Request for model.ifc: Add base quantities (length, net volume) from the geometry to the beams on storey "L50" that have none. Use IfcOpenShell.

First a look at what the model holds.

```python
import ifcopenshell
import ifcopenshell.util.element
import ifcopenshell.util.unit

model = ifcopenshell.open("model.ifc")
print(model.schema)
for unit_type in ("LENGTHUNIT", "AREAUNIT", "VOLUMEUNIT"):
    print(unit_type, ifcopenshell.util.unit.calculate_unit_scale(model, unit_type))
storey = next(s for s in model.by_type("IfcBuildingStorey") if s.Name == "L50")
beams = [e for e in ifcopenshell.util.element.get_decomposition(storey) if e.is_a("IfcBeam")]
for e in sorted(beams, key=lambda e: e.id()):
    print(e.id(), e.is_a(), e.Name, list(ifcopenshell.util.element.get_psets(e, qtos_only=True)), sep=" | ")
```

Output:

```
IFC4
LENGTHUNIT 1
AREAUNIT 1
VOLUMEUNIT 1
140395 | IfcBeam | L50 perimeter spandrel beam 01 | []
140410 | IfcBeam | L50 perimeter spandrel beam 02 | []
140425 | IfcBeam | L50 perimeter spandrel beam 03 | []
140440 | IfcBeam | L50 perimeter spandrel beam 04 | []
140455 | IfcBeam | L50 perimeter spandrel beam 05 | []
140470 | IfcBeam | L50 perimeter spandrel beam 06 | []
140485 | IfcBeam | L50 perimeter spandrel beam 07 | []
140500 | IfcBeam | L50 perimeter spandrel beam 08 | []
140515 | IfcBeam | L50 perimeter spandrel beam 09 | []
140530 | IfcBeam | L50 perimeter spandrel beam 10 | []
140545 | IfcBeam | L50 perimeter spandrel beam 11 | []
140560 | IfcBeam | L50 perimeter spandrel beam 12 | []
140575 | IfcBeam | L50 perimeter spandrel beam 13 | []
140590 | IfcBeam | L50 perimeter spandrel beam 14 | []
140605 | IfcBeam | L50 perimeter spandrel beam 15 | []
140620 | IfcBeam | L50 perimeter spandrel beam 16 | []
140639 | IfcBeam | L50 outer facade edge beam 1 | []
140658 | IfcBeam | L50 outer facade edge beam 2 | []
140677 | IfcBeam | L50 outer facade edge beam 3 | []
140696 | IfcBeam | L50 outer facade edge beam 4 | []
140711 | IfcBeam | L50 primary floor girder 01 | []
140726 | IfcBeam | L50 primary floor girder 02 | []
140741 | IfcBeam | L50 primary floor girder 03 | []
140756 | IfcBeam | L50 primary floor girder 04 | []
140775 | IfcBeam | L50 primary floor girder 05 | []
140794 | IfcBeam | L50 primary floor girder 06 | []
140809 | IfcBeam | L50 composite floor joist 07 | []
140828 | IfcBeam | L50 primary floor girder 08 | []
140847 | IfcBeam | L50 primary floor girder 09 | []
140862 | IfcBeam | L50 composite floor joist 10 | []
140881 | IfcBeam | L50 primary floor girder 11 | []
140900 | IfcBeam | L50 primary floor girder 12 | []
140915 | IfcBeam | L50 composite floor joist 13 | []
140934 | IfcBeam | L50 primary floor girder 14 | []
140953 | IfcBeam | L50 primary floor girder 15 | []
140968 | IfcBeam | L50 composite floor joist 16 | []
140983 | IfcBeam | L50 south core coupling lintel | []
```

```python
import ifcopenshell
import ifcopenshell.api.pset
import ifcopenshell.geom
import ifcopenshell.util.element
import ifcopenshell.util.shape
import ifcopenshell.util.unit

model = ifcopenshell.open("model.ifc")
unit_scale = ifcopenshell.util.unit.calculate_unit_scale(model)
volume_scale = ifcopenshell.util.unit.calculate_unit_scale(model, "VOLUMEUNIT")
settings = ifcopenshell.geom.settings()

storey = next(s for s in model.by_type("IfcBuildingStorey") if s.Name == "L50")
beams = [e for e in ifcopenshell.util.element.get_decomposition(storey) if e.is_a("IfcBeam")]

for e in sorted(beams, key=lambda e: e.id()):
    if ifcopenshell.util.element.get_psets(e, qtos_only=True, should_inherit=False):
        continue
    # Geometry comes back in metres, in the element's own axes.
    shape = ifcopenshell.geom.create_shape(settings, e)
    values = {
        "Length": ifcopenshell.util.shape.get_max_xyz(shape.geometry) / unit_scale,
        "NetVolume": ifcopenshell.util.shape.get_volume(shape.geometry) / volume_scale,
    }
    qto = ifcopenshell.api.pset.add_qto(model, product=e, name="Qto_BeamBaseQuantities")
    ifcopenshell.api.pset.edit_qto(model, qto=qto, properties=values)
    print(e.id(), {k: round(v, 3) for k, v in values.items()})

model.write("model_edited.ifc")
```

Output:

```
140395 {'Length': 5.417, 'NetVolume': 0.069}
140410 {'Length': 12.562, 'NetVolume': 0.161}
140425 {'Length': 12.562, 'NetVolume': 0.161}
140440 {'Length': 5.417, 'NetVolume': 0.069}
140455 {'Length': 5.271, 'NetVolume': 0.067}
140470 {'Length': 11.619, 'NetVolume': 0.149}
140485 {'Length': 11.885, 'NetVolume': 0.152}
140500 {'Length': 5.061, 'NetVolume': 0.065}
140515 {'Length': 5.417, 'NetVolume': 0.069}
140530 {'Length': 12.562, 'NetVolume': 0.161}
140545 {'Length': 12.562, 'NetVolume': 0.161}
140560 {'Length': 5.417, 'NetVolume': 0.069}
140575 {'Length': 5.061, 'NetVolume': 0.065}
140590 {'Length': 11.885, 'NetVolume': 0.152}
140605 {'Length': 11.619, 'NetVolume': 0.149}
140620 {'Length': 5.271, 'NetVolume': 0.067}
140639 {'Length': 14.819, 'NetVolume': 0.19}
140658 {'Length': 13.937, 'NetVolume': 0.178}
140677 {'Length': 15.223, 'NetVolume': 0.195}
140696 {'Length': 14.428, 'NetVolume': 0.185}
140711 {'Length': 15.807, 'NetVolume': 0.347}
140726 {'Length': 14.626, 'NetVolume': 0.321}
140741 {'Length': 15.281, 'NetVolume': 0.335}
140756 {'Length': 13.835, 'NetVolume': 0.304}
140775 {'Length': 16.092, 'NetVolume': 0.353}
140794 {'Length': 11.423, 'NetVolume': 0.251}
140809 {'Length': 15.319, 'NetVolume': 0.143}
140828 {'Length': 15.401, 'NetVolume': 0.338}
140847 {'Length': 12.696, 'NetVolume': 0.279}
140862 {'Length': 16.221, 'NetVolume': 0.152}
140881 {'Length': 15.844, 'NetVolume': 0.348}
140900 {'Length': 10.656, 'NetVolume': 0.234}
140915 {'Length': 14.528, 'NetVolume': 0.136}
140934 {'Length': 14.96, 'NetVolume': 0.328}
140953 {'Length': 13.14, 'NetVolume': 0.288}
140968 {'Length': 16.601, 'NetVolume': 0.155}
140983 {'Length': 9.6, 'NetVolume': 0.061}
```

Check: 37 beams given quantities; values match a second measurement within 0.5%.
